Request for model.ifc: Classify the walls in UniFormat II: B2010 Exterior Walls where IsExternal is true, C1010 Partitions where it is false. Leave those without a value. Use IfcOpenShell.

First a look at what the model holds.

```python
import ifcopenshell
import ifcopenshell.util.element

model = ifcopenshell.open("model.ifc")
print(model.schema)
print("classifications:", [c.Name for c in model.by_type("IfcClassification")])
values = [ifcopenshell.util.element.get_pset(e, "Pset_WallCommon", "IsExternal") for e in model.by_type("IfcWall")]
for value in (True, False, None):
    print("IsExternal", value, values.count(value))
```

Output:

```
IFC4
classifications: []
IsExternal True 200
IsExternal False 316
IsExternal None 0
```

```python
import ifcopenshell
import ifcopenshell.api.classification
import ifcopenshell.util.element

model = ifcopenshell.open("model.ifc")

system = ifcopenshell.api.classification.add_classification(model, classification="UniFormat II")

walls = model.by_type("IfcWall")
external = {e: ifcopenshell.util.element.get_pset(e, "Pset_WallCommon", "IsExternal") for e in walls}
for flag, code, name in ((True, "B2010", "Exterior Walls"), (False, "C1010", "Partitions")):
    products = [e for e in walls if external[e] is flag]
    ifcopenshell.api.classification.add_reference(
        model, products=products, classification=system, identification=code, name=name
    )
    print(code, len(products))

model.write("model_edited.ifc")
```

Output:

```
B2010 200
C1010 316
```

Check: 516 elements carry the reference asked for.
